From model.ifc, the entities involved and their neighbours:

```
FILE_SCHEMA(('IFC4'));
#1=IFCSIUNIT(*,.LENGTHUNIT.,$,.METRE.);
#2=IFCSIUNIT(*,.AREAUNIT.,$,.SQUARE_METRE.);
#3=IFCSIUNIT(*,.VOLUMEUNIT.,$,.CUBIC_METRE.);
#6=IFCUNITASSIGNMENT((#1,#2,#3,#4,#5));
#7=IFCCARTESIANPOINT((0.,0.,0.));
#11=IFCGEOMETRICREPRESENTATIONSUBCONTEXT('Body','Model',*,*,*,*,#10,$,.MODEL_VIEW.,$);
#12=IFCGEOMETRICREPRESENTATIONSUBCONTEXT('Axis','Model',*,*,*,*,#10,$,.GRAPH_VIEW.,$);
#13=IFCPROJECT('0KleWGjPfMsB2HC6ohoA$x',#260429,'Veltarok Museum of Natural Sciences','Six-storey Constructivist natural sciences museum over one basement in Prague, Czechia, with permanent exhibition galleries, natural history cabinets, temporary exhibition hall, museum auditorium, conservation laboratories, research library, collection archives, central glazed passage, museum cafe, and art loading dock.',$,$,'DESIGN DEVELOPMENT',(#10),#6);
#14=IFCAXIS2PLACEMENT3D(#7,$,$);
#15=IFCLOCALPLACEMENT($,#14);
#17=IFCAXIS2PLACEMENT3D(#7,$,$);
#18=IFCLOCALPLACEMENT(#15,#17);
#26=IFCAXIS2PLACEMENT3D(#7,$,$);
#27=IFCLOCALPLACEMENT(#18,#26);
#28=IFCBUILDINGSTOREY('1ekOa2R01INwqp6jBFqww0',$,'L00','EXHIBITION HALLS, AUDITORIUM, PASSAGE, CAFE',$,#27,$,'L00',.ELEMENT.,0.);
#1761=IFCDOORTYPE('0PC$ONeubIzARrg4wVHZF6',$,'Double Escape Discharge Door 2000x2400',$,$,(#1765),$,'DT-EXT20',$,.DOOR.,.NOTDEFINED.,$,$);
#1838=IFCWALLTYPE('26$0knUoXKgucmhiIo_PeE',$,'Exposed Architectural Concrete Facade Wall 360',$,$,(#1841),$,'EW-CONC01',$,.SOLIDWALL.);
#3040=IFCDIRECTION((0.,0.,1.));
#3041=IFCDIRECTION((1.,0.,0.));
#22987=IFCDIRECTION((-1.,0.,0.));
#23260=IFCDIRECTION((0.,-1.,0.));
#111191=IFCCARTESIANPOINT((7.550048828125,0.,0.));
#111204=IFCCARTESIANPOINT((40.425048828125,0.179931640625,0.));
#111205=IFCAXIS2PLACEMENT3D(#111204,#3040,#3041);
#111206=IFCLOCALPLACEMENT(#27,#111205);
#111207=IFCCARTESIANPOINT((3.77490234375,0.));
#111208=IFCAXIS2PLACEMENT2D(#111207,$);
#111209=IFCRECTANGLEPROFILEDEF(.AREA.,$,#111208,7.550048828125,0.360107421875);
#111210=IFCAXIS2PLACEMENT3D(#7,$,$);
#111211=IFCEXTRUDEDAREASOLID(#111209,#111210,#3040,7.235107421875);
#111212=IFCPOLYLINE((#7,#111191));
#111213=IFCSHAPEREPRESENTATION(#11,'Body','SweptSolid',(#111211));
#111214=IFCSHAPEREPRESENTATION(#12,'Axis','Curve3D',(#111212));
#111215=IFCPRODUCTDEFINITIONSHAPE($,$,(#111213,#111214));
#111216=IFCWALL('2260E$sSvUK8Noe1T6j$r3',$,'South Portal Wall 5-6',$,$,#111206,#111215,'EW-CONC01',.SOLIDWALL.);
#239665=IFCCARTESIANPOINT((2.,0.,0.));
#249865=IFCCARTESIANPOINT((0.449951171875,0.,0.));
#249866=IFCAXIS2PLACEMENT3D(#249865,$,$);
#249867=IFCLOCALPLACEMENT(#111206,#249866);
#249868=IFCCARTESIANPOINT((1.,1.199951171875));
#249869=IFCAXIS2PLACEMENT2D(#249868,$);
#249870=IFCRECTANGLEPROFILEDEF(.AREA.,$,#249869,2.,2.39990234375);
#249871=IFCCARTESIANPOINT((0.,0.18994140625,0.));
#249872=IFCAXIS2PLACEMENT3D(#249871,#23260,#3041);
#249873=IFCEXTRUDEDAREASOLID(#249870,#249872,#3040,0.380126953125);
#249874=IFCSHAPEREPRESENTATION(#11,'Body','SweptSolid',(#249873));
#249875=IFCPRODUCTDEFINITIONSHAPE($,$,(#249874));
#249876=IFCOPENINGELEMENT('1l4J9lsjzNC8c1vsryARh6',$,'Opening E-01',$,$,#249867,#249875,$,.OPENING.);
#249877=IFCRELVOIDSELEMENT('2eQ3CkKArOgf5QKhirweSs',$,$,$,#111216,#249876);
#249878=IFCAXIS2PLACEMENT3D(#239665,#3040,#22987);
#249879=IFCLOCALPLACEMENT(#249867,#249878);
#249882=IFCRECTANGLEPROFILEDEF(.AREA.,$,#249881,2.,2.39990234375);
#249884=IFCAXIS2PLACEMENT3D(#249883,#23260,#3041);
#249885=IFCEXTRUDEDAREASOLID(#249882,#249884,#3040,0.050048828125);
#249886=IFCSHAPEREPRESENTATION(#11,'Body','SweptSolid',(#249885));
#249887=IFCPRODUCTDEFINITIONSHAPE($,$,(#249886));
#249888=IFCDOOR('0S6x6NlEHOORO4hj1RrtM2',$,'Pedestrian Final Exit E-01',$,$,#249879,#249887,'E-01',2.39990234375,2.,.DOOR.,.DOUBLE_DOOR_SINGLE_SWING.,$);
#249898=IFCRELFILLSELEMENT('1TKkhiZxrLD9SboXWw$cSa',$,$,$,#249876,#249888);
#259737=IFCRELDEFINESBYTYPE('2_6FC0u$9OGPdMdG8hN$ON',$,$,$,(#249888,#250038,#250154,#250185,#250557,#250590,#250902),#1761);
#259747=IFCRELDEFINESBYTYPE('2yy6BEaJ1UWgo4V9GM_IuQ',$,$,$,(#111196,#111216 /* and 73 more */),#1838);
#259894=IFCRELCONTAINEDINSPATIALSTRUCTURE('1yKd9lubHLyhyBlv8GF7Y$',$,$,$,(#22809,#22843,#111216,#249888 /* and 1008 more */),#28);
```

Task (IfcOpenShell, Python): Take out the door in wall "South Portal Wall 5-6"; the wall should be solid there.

```python
import ifcopenshell
import ifcopenshell.api.feature
import ifcopenshell.api.root
import ifcopenshell.geom
import ifcopenshell.util.shape

model = ifcopenshell.open("model.ifc")
settings = ifcopenshell.geom.settings()


def volume(element):
    """Net volume in cubic metres, openings subtracted."""
    shape = ifcopenshell.geom.create_shape(settings, element)
    return ifcopenshell.util.shape.get_volume(shape.geometry)


door = model.by_guid("0S6x6NlEHOORO4hj1RrtM2")
opening = door.FillsVoids[0].RelatingOpeningElement
wall = opening.VoidsElements[0].RelatingBuildingElement
before = volume(wall)

ifcopenshell.api.root.remove_product(model, product=door)
ifcopenshell.api.feature.remove_feature(model, feature=opening)

after = volume(wall)

print(f"wall volume {before:.3f} -> {after:.3f} m3")

model.write("model_rev.ifc")
```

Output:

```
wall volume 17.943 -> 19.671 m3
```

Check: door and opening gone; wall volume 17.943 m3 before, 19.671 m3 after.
